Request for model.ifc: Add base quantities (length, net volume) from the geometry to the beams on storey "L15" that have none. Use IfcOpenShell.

First a look at what the model holds.

```python
import ifcopenshell
import ifcopenshell.util.element
import ifcopenshell.util.unit

model = ifcopenshell.open("model.ifc")
print(model.schema)
for unit_type in ("LENGTHUNIT", "AREAUNIT", "VOLUMEUNIT"):
    print(unit_type, ifcopenshell.util.unit.calculate_unit_scale(model, unit_type))
storey = next(s for s in model.by_type("IfcBuildingStorey") if s.Name == "L15")
beams = [e for e in ifcopenshell.util.element.get_decomposition(storey) if e.is_a("IfcBeam")]
for e in sorted(beams, key=lambda e: e.id()):
    print(e.id(), e.is_a(), e.Name, list(ifcopenshell.util.element.get_psets(e, qtos_only=True)), sep=" | ")
```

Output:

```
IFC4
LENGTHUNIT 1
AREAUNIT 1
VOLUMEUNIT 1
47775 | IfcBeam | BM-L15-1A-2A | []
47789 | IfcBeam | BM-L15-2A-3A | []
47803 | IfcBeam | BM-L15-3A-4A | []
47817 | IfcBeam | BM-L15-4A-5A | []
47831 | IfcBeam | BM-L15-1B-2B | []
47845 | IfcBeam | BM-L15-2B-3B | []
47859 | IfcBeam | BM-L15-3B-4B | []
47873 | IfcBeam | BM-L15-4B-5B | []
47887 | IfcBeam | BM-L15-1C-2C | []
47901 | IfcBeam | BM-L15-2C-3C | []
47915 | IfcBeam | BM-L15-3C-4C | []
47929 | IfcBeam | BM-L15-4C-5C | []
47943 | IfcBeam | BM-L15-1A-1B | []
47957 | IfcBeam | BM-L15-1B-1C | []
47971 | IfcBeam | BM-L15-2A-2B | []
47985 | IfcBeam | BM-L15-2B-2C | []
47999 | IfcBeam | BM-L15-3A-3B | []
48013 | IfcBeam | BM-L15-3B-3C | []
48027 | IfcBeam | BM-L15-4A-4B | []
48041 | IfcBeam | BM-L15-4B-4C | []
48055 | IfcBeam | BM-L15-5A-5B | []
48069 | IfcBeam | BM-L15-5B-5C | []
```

```python
import ifcopenshell
import ifcopenshell.api.pset
import ifcopenshell.geom
import ifcopenshell.util.element
import ifcopenshell.util.shape
import ifcopenshell.util.unit

model = ifcopenshell.open("model.ifc")
unit_scale = ifcopenshell.util.unit.calculate_unit_scale(model)
volume_scale = ifcopenshell.util.unit.calculate_unit_scale(model, "VOLUMEUNIT")
settings = ifcopenshell.geom.settings()

storey = next(s for s in model.by_type("IfcBuildingStorey") if s.Name == "L15")
beams = [e for e in ifcopenshell.util.element.get_decomposition(storey) if e.is_a("IfcBeam")]

for e in sorted(beams, key=lambda e: e.id()):
    if ifcopenshell.util.element.get_psets(e, qtos_only=True, should_inherit=False):
        continue
    # Geometry comes back in metres, in the element's own axes.
    shape = ifcopenshell.geom.create_shape(settings, e)
    values = {
        "Length": ifcopenshell.util.shape.get_max_xyz(shape.geometry) / unit_scale,
        "NetVolume": ifcopenshell.util.shape.get_volume(shape.geometry) / volume_scale,
    }
    qto = ifcopenshell.api.pset.add_qto(model, product=e, name="Qto_BeamBaseQuantities")
    ifcopenshell.api.pset.edit_qto(model, qto=qto, properties=values)
    print(e.id(), {k: round(v, 3) for k, v in values.items()})

model.write("model_v2.ifc")
```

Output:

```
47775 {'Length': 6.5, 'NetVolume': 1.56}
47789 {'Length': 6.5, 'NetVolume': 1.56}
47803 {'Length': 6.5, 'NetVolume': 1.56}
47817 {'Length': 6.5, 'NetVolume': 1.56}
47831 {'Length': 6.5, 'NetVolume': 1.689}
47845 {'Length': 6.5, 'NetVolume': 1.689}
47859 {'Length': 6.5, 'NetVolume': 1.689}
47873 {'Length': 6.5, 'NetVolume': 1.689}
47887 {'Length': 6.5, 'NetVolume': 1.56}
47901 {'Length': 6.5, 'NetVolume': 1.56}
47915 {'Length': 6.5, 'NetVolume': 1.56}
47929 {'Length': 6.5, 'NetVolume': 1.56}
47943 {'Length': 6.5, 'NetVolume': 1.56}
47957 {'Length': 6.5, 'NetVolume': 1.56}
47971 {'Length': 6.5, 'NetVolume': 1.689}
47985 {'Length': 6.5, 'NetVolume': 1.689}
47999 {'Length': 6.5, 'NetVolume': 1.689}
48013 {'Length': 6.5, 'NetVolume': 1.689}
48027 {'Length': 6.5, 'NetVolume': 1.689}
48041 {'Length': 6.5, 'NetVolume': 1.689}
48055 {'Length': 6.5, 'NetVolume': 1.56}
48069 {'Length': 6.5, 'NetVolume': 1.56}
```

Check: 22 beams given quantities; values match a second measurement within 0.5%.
